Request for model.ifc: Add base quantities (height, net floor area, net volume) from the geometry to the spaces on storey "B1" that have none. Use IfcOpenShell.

First a look at what the model holds.

```python
import ifcopenshell
import ifcopenshell.util.element
import ifcopenshell.util.unit

model = ifcopenshell.open("model.ifc")
print(model.schema)
for unit_type in ("LENGTHUNIT", "AREAUNIT", "VOLUMEUNIT"):
    print(unit_type, ifcopenshell.util.unit.calculate_unit_scale(model, unit_type))
storey = next(s for s in model.by_type("IfcBuildingStorey") if s.Name == "B1")
spaces = [e for e in ifcopenshell.util.element.get_decomposition(storey) if e.is_a("IfcSpace")]
for e in sorted(spaces, key=lambda e: e.id()):
    print(e.id(), e.is_a(), e.Name, list(ifcopenshell.util.element.get_psets(e, qtos_only=True)), sep=" | ")
```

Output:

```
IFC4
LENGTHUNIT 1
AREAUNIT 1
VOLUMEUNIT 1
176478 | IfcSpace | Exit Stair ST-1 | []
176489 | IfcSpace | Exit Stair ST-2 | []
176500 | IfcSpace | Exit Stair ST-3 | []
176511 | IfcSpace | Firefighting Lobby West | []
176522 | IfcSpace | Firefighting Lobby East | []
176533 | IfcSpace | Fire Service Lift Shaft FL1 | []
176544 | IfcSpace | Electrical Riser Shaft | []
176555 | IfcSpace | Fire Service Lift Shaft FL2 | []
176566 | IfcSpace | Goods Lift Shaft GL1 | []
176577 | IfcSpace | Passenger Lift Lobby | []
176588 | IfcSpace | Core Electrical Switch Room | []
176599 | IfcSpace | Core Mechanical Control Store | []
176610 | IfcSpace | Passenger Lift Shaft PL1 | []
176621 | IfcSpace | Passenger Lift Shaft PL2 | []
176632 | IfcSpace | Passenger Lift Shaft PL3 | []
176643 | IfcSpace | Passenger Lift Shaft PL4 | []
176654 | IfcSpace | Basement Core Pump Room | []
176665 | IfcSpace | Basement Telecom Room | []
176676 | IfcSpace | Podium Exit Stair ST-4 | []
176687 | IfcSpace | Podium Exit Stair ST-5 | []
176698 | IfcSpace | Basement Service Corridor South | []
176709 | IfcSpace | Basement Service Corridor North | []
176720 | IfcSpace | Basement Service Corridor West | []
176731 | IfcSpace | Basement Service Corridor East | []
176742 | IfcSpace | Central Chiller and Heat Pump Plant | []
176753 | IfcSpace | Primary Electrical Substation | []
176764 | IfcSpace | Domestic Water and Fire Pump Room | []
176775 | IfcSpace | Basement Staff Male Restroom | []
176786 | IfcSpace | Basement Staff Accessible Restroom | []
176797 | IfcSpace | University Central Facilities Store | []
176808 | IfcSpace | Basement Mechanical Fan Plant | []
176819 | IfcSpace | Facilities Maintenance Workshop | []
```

```python
import ifcopenshell
import ifcopenshell.api.pset
import ifcopenshell.geom
import ifcopenshell.util.element
import ifcopenshell.util.shape
import ifcopenshell.util.unit

model = ifcopenshell.open("model.ifc")
unit_scale = ifcopenshell.util.unit.calculate_unit_scale(model)
area_scale = ifcopenshell.util.unit.calculate_unit_scale(model, "AREAUNIT")
volume_scale = ifcopenshell.util.unit.calculate_unit_scale(model, "VOLUMEUNIT")
settings = ifcopenshell.geom.settings()

storey = next(s for s in model.by_type("IfcBuildingStorey") if s.Name == "B1")
spaces = [e for e in ifcopenshell.util.element.get_decomposition(storey) if e.is_a("IfcSpace")]

for e in sorted(spaces, key=lambda e: e.id()):
    if ifcopenshell.util.element.get_psets(e, qtos_only=True, should_inherit=False):
        continue
    # Geometry comes back in metres, in the element's own axes.
    shape = ifcopenshell.geom.create_shape(settings, e)
    values = {
        "Height": ifcopenshell.util.shape.get_z(shape.geometry) / unit_scale,
        "NetFloorArea": ifcopenshell.util.shape.get_footprint_area(shape.geometry) / area_scale,
        "NetVolume": ifcopenshell.util.shape.get_volume(shape.geometry) / volume_scale,
    }
    qto = ifcopenshell.api.pset.add_qto(model, product=e, name="Qto_SpaceBaseQuantities")
    ifcopenshell.api.pset.edit_qto(model, qto=qto, properties=values)
    print(e.id(), {k: round(v, 3) for k, v in values.items()})

model.write("model_edited.ifc")
```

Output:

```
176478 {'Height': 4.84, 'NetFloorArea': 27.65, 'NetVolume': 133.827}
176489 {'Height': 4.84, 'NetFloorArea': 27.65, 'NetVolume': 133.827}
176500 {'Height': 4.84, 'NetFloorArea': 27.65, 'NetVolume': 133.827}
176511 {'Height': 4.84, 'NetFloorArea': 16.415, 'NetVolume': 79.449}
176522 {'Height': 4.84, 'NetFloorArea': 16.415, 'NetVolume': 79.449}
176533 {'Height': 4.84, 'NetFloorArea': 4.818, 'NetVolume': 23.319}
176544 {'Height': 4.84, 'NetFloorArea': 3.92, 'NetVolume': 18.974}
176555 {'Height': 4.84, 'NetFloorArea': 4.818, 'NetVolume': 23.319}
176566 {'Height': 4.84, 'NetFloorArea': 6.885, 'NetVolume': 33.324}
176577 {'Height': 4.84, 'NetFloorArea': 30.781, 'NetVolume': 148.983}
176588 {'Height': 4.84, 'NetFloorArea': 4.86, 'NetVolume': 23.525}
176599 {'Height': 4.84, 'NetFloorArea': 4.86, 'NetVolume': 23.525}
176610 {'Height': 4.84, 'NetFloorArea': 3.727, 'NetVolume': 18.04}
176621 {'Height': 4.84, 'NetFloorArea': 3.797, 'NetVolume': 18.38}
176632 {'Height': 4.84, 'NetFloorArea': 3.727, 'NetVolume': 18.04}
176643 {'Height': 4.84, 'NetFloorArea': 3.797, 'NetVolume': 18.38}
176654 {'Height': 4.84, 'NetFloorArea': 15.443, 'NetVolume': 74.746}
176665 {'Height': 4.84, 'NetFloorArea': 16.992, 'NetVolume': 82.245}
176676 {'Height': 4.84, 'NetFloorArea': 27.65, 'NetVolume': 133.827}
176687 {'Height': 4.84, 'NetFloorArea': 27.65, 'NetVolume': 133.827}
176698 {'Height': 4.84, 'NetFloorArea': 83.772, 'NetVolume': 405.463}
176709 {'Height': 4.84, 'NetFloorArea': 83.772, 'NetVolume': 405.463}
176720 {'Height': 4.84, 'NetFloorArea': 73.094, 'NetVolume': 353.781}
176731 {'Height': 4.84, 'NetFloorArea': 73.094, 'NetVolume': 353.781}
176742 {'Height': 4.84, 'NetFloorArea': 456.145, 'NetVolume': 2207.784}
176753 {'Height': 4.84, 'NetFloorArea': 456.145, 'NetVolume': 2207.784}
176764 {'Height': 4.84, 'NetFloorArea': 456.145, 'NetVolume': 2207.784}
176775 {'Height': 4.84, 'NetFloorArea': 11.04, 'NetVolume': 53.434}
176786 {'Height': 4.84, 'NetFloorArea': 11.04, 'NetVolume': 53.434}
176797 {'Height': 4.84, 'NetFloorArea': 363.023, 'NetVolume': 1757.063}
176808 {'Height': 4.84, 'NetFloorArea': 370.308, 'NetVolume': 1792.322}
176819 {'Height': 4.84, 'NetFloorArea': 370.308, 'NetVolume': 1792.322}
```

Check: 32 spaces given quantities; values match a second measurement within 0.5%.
